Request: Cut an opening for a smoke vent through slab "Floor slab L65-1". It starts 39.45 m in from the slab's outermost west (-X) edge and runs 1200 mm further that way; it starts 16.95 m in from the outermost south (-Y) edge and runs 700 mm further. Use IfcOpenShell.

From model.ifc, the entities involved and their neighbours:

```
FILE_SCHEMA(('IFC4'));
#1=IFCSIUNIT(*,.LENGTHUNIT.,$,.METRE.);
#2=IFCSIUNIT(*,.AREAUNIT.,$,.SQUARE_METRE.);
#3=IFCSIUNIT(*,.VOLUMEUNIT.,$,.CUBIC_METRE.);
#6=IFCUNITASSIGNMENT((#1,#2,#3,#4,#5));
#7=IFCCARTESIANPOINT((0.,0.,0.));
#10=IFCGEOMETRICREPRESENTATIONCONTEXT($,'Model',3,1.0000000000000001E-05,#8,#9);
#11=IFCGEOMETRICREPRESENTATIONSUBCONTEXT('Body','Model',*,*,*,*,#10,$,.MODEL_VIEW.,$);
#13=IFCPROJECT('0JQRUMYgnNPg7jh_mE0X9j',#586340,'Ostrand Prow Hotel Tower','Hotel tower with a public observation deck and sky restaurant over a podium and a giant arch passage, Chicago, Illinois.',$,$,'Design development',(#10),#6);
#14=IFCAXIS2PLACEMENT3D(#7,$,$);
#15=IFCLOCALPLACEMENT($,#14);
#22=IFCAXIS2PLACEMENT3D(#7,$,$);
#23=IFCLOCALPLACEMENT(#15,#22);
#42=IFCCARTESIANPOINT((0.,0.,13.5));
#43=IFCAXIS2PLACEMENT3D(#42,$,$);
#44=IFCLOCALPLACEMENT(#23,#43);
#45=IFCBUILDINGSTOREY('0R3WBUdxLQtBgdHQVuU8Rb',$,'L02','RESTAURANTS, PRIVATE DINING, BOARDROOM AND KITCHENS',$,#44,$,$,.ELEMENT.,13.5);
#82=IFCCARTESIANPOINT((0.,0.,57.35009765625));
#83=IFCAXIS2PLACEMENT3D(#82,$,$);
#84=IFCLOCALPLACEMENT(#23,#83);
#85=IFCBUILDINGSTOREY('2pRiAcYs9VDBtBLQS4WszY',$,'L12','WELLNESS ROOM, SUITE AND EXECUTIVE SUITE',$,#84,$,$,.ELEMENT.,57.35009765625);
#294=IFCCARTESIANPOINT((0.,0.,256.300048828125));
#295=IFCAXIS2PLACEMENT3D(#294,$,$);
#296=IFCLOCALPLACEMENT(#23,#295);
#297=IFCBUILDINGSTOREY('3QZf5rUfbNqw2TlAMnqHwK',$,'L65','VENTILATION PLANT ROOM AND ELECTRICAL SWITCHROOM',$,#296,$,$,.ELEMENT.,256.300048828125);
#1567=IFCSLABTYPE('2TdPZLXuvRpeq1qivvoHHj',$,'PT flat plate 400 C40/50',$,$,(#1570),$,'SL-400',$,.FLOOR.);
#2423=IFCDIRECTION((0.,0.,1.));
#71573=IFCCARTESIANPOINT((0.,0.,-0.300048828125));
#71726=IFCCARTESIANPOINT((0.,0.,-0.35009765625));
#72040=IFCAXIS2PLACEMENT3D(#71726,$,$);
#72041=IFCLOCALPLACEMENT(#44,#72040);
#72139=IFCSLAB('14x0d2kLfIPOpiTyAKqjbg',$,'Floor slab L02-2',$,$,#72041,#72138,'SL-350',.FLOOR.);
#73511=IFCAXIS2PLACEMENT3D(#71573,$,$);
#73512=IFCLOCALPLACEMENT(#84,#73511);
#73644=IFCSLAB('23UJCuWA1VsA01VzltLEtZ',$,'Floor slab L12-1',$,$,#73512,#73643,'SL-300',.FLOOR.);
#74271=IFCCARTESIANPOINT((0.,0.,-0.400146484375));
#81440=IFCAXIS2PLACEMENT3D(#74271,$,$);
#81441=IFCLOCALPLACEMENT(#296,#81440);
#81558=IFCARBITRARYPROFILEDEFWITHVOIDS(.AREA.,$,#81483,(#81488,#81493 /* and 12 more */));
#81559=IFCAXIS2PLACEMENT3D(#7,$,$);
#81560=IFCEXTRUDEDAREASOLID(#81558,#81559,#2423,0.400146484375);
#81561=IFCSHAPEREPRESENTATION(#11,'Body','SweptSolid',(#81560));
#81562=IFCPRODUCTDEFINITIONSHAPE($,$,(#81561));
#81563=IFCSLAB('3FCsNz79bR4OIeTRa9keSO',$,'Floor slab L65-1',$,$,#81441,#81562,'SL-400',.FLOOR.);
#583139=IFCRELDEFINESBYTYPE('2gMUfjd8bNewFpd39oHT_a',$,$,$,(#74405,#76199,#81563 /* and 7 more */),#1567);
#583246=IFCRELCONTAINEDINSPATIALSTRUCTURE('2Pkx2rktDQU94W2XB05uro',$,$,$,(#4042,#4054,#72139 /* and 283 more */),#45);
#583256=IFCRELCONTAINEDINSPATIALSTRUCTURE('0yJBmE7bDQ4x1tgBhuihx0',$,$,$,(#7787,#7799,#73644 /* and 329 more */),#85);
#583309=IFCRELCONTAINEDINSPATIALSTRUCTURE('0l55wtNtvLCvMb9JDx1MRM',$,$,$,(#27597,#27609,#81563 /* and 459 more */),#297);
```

```python
import numpy as np
import ifcopenshell
import ifcopenshell.api.feature
import ifcopenshell.api.geometry
import ifcopenshell.api.root
import ifcopenshell.geom
import ifcopenshell.util.placement
import ifcopenshell.util.representation
import ifcopenshell.util.shape
import ifcopenshell.util.unit

model = ifcopenshell.open("model.ifc")
unit_scale = ifcopenshell.util.unit.calculate_unit_scale(model)
settings = ifcopenshell.geom.settings()


def volume(element):
    """Net volume in cubic metres, openings subtracted."""
    shape = ifcopenshell.geom.create_shape(settings, element)
    return ifcopenshell.util.shape.get_volume(shape.geometry)


slab = model.by_id(81563)
before = volume(slab)

# Extent in the slab's own axes, in metres. The edges named are its -X and -Y sides.
slab_shape = ifcopenshell.geom.create_shape(settings, slab)
vertices = ifcopenshell.util.shape.get_vertices(slab_shape.geometry)
x_min, y_min, bottom = vertices.min(axis=0)
top = vertices[:, 2].max()

opening = ifcopenshell.api.root.create_entity(model, ifc_class="IfcOpeningElement", name="Smoke vent opening", predefined_type="OPENING")
context = ifcopenshell.util.representation.get_context(model, "Model", "Body", "MODEL_VIEW")
width, depth = 1.2, 0.7
outline = [(0.0, 0.0), (width, 0.0), (width, depth), (0.0, depth), (0.0, 0.0)]
# Overshoot both faces by 50 mm so the cut is clean.
shape = ifcopenshell.api.geometry.add_slab_representation(
    model, context=context, depth=top - bottom + 0.1, polyline=outline
)
ifcopenshell.api.geometry.assign_representation(model, product=opening, representation=shape)

matrix = ifcopenshell.util.placement.get_local_placement(slab.ObjectPlacement)
matrix[:, 3] = matrix @ np.append(np.array([x_min + 39.45, y_min + 16.95, bottom - 0.05]) / unit_scale, 1.0)
ifcopenshell.api.geometry.edit_object_placement(model, product=opening, matrix=matrix, is_si=False)
ifcopenshell.api.feature.add_feature(model, feature=opening, element=slab)

after = volume(slab)

print(f"slab volume {before:.3f} -> {after:.3f} m3")

model.write("model_updated.ifc")
```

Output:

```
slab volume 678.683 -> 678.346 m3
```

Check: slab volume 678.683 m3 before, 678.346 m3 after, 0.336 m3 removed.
